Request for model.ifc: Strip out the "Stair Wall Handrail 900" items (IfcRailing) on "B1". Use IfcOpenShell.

First a look at what the model holds.

```python
import ifcopenshell
import ifcopenshell.util.element

model = ifcopenshell.open("model.ifc")
print(model.schema)
storey = next(s for s in model.by_type("IfcBuildingStorey") if s.Name == "B1")
railings = [e for e in ifcopenshell.util.element.get_decomposition(storey) if e.is_a("IfcRailing")]
seen = {}
for e in railings:
    element_type = ifcopenshell.util.element.get_type(e)
    name = element_type.Name if element_type not in (None, e) else None
    seen[name] = seen.get(name, 0) + 1
for name, count in sorted(seen.items(), key=str):
    print(count, "x", name)
```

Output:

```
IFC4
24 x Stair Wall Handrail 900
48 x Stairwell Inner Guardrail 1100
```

```python
import ifcopenshell
import ifcopenshell.api.root
import ifcopenshell.util.element

model = ifcopenshell.open("model.ifc")

storey = next(s for s in model.by_type("IfcBuildingStorey") if s.Name == "B1")
railings = [e for e in ifcopenshell.util.element.get_decomposition(storey) if e.is_a("IfcRailing")]
targets = [e for e in railings if (t := ifcopenshell.util.element.get_type(e)) not in (None, e) and t.Name == "Stair Wall Handrail 900"]

for e in targets:
    ifcopenshell.api.root.remove_product(model, product=e)
print(len(targets), "removed")

model.write("model_v2.ifc")
```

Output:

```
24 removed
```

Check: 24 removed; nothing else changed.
